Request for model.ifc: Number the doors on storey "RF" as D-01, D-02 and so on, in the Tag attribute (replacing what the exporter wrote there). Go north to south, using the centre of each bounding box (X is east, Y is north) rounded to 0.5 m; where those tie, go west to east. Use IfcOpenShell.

First a look at what the model holds.

```python
import ifcopenshell
import ifcopenshell.util.element
import ifcopenshell.util.placement

model = ifcopenshell.open("model.ifc")
print(model.schema)
storey = next(s for s in model.by_type("IfcBuildingStorey") if s.Name == "RF")
doors = [e for e in ifcopenshell.util.element.get_decomposition(storey) if e.is_a("IfcDoor")]
for e in sorted(doors, key=lambda e: e.id()):
    origin = ifcopenshell.util.placement.get_local_placement(e.ObjectPlacement)[:3, 3]
    print(e.id(), e.Tag, e.Name, origin.round(2) + 0.0, sep=" | ")
```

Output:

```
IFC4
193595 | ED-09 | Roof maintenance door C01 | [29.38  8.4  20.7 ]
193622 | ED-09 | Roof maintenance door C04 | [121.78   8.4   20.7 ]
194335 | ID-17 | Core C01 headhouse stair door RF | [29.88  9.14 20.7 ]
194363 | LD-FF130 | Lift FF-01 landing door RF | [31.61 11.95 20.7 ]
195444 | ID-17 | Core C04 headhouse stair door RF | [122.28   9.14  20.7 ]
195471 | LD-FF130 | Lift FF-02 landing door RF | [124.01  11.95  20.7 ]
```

```python
import ifcopenshell
import ifcopenshell.geom
import ifcopenshell.util.element
import ifcopenshell.util.shape

model = ifcopenshell.open("model.ifc")
settings = ifcopenshell.geom.settings()
settings.set("use-world-coords", True)


def centre(element):
    shape = ifcopenshell.geom.create_shape(settings, element)
    return ifcopenshell.util.shape.get_bbox_centroid(shape.geometry)


storey = next(s for s in model.by_type("IfcBuildingStorey") if s.Name == "RF")
doors = [e for e in ifcopenshell.util.element.get_decomposition(storey) if e.is_a("IfcDoor")]

# Insertion points can sit at a corner or the storey origin, so sort by the geometry (in metres).
centres = {e: centre(e) for e in doors}
doors.sort(key=lambda e: (-round(centres[e][1] / 0.5), centres[e][0]))

for i, e in enumerate(doors, start=1):
    number = f"D-{i:02d}"
    e.Tag = number
    print(e.id(), number)

model.write("model_rev.ifc")
```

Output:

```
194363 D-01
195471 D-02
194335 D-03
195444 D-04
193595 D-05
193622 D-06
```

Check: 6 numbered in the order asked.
